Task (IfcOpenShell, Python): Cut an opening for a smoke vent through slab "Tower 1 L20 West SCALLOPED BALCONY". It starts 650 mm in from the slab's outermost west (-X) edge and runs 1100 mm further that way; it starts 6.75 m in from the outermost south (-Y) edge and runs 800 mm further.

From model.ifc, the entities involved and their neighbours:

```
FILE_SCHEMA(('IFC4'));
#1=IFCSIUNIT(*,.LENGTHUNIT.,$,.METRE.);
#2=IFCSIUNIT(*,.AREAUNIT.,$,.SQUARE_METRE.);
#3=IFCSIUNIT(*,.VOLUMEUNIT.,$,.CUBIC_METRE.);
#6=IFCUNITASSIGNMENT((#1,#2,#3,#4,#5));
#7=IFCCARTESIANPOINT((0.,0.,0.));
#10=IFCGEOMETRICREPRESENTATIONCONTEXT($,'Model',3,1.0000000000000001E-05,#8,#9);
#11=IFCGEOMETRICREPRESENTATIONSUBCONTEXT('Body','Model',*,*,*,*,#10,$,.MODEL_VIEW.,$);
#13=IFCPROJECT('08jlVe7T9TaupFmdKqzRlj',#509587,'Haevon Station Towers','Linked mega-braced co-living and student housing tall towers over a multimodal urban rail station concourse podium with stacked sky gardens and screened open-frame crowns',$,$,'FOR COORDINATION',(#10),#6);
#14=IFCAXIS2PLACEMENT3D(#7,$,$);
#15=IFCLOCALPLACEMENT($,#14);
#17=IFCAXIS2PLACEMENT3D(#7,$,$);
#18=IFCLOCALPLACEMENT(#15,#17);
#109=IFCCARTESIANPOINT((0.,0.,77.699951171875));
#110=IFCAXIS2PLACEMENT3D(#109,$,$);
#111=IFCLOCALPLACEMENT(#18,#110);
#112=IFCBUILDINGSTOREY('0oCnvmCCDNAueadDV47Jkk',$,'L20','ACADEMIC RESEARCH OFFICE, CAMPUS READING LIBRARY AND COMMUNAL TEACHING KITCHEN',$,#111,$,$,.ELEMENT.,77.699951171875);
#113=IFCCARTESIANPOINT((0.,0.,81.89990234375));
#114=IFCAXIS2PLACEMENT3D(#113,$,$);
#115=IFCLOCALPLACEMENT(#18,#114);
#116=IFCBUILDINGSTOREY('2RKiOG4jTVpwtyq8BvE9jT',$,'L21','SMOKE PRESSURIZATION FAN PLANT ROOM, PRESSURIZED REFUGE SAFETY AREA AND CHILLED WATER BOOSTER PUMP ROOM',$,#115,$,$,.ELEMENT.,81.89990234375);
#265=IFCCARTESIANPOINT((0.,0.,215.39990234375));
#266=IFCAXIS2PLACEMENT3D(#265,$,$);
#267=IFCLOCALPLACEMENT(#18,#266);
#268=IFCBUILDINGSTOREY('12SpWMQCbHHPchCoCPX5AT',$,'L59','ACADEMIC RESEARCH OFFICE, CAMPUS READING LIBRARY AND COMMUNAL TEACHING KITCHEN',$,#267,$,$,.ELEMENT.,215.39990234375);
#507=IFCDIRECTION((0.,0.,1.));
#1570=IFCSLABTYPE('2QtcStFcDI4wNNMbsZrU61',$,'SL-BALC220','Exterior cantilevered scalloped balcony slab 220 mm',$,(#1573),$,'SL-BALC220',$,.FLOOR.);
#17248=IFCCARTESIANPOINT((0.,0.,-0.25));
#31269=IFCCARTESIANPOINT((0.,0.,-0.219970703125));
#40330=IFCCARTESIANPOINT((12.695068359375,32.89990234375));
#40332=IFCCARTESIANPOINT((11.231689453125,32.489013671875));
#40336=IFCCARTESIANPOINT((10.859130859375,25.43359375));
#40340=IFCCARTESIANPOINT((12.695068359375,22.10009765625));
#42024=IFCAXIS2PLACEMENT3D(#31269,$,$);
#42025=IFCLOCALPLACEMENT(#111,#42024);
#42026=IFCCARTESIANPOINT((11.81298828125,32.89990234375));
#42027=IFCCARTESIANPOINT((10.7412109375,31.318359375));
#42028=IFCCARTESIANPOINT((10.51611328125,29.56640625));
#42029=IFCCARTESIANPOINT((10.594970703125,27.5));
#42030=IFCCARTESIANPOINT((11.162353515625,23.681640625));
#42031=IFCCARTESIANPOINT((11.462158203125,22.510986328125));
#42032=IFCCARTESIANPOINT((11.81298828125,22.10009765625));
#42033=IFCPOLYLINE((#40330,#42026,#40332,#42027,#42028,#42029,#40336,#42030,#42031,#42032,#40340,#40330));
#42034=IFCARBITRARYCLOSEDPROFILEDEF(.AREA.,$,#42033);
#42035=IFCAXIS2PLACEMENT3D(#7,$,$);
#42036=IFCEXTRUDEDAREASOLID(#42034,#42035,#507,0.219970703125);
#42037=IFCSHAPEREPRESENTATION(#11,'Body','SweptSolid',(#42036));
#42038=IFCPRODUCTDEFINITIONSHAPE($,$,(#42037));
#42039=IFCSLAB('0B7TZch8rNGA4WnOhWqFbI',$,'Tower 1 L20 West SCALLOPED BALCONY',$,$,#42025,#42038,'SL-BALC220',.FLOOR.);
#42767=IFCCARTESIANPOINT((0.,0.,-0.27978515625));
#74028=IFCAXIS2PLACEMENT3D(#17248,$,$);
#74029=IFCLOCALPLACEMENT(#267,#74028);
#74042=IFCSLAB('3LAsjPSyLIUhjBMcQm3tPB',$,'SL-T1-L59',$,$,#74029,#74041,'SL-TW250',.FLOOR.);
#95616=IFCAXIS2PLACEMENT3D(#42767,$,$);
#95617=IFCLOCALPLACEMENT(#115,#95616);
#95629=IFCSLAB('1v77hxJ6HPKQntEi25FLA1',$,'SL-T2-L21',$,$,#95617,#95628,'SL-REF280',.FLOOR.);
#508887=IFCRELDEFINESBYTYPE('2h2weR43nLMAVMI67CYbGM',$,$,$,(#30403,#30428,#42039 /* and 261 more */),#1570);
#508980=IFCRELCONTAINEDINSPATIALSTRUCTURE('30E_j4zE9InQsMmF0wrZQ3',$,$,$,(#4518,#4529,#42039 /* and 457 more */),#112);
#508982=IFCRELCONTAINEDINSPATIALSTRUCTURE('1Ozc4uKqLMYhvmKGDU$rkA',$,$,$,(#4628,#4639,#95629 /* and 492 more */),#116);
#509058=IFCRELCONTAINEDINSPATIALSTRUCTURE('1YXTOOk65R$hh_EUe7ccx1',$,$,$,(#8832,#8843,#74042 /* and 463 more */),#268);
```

```python
import numpy as np
import ifcopenshell
import ifcopenshell.api.feature
import ifcopenshell.api.geometry
import ifcopenshell.api.root
import ifcopenshell.geom
import ifcopenshell.util.placement
import ifcopenshell.util.representation
import ifcopenshell.util.shape
import ifcopenshell.util.unit

model = ifcopenshell.open("model.ifc")
unit_scale = ifcopenshell.util.unit.calculate_unit_scale(model)
settings = ifcopenshell.geom.settings()


def volume(element):
    """Net volume in cubic metres, openings subtracted."""
    shape = ifcopenshell.geom.create_shape(settings, element)
    return ifcopenshell.util.shape.get_volume(shape.geometry)


slab = model.by_guid("0B7TZch8rNGA4WnOhWqFbI")
before = volume(slab)

# Extent in the slab's own axes, in metres. The edges named are its -X and -Y sides.
slab_shape = ifcopenshell.geom.create_shape(settings, slab)
vertices = ifcopenshell.util.shape.get_vertices(slab_shape.geometry)
x_min, y_min, bottom = vertices.min(axis=0)
top = vertices[:, 2].max()

opening = ifcopenshell.api.root.create_entity(model, ifc_class="IfcOpeningElement", name="Smoke vent opening", predefined_type="OPENING")
context = ifcopenshell.util.representation.get_context(model, "Model", "Body", "MODEL_VIEW")
width, depth = 1.1, 0.8
outline = [(0.0, 0.0), (width, 0.0), (width, depth), (0.0, depth), (0.0, 0.0)]
# Overshoot both faces by 50 mm so the cut is clean.
shape = ifcopenshell.api.geometry.add_slab_representation(
    model, context=context, depth=top - bottom + 0.1, polyline=outline
)
ifcopenshell.api.geometry.assign_representation(model, product=opening, representation=shape)

matrix = ifcopenshell.util.placement.get_local_placement(slab.ObjectPlacement)
matrix[:, 3] = matrix @ np.append(np.array([x_min + 0.65, y_min + 6.75, bottom - 0.05]) / unit_scale, 1.0)
ifcopenshell.api.geometry.edit_object_placement(model, product=opening, matrix=matrix, is_si=False)
ifcopenshell.api.feature.add_feature(model, feature=opening, element=slab)

after = volume(slab)

print(f"slab volume {before:.3f} -> {after:.3f} m3")

model.write("model_edited.ifc")
```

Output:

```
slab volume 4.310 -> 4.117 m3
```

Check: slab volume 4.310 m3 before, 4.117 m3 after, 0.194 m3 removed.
